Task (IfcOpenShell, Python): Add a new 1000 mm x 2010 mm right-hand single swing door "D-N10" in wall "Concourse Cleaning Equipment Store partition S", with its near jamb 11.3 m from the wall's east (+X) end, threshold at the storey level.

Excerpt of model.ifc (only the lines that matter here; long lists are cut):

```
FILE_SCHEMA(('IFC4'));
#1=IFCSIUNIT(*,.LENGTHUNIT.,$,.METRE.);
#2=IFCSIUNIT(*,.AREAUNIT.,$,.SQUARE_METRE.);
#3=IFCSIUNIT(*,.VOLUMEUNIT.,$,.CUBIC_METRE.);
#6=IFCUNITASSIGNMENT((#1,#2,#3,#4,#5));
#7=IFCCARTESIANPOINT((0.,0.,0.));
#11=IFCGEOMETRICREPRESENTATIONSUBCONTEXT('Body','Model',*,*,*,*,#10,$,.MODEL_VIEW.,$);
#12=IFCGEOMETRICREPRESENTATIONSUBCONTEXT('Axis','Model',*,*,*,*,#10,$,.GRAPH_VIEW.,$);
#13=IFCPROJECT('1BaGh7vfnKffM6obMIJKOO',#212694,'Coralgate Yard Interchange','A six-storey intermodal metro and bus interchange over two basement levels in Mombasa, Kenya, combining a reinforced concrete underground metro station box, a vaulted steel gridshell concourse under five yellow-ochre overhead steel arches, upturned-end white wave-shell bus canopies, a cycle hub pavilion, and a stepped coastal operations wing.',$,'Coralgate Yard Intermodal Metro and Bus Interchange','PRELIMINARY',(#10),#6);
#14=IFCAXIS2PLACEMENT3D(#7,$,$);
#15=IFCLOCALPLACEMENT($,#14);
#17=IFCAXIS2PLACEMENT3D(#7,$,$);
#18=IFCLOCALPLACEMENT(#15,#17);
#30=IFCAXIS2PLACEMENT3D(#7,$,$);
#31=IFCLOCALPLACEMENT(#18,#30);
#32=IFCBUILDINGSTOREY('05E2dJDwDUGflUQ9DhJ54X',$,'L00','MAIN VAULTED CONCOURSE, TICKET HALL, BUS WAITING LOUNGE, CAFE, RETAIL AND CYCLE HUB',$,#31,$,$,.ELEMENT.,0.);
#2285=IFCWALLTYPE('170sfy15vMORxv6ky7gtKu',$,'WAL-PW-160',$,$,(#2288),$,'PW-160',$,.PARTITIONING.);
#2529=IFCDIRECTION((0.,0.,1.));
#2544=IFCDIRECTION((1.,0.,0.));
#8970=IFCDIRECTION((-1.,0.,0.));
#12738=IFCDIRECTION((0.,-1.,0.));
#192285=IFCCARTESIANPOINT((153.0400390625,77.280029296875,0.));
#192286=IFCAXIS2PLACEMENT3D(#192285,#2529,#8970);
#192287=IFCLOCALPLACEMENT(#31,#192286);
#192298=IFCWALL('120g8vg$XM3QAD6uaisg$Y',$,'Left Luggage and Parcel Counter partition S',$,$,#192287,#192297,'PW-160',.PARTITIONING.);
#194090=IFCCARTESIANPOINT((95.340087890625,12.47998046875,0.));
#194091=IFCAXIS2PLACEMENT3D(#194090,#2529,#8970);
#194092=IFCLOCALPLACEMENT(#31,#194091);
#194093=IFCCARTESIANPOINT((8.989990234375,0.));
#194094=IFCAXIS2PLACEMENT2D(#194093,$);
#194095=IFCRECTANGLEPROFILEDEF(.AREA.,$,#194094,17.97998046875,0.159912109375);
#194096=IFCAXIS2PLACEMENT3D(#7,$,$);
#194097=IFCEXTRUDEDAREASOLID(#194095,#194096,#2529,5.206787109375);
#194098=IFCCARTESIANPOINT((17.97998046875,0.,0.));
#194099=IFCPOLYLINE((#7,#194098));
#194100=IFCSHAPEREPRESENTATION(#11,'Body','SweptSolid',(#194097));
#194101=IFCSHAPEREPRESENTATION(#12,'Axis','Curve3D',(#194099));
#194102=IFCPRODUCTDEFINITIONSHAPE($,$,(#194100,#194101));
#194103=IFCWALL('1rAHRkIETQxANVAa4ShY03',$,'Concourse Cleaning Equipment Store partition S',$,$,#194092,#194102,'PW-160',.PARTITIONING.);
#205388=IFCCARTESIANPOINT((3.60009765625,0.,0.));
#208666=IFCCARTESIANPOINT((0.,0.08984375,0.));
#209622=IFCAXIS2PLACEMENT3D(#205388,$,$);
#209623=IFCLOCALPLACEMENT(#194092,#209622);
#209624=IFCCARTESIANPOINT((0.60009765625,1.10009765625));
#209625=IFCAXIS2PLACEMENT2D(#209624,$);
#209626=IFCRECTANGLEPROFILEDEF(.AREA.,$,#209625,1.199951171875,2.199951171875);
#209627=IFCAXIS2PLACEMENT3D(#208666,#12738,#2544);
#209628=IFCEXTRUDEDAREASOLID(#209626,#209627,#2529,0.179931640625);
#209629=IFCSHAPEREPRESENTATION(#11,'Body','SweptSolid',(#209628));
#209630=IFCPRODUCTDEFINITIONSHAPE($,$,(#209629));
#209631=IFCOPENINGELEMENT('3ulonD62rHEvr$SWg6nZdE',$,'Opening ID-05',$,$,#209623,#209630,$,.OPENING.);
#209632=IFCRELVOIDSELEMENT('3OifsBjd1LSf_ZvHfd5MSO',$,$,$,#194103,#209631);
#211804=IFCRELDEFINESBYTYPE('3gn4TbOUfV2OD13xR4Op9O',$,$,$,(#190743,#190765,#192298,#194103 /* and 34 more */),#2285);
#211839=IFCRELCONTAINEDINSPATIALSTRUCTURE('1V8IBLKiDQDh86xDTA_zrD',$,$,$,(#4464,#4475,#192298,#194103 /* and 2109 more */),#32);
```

```python
import numpy as np
import ifcopenshell
import ifcopenshell.api.feature
import ifcopenshell.api.geometry
import ifcopenshell.api.root
import ifcopenshell.api.spatial
import ifcopenshell.geom
import ifcopenshell.util.element
import ifcopenshell.util.placement
import ifcopenshell.util.representation
import ifcopenshell.util.shape
import ifcopenshell.util.unit

model = ifcopenshell.open("model.ifc")
unit_scale = ifcopenshell.util.unit.calculate_unit_scale(model)
settings = ifcopenshell.geom.settings()


def volume(element):
    """Net volume in cubic metres, openings subtracted."""
    shape = ifcopenshell.geom.create_shape(settings, element)
    return ifcopenshell.util.shape.get_volume(shape.geometry)


wall = model.by_id(194103)
storey = ifcopenshell.util.element.get_container(wall, ifc_class="IfcBuildingStorey")
context = ifcopenshell.util.representation.get_context(model, "Model", "Body", "MODEL_VIEW")
before = volume(wall)

width, height, from_end, sill = 1, 2.01, 11.3, 0.0  # metres

# The wall runs along its own X axis, and the end named is its -X end.
wall_shape = ifcopenshell.geom.create_shape(settings, wall)
x, y, z = ifcopenshell.util.shape.get_vertices(wall_shape.geometry).T
start = x.min() + from_end
face, thickness = float(y.min()), float(y.max() - y.min())
wall_matrix = ifcopenshell.util.placement.get_local_placement(wall.ObjectPlacement)
level = ifcopenshell.util.placement.get_local_placement(storey.ObjectPlacement)[2, 3]


def in_wall(x, y):
    """Placement at x, y metres in the wall's axes, at sill height."""
    matrix = wall_matrix.copy()
    matrix[:, 3] = wall_matrix @ np.array([x / unit_scale, y / unit_scale, 0.0, 1.0])
    matrix[2, 3] = level + sill / unit_scale
    return matrix


# Opening: a box that overshoots both wall faces by 50 mm.
opening = ifcopenshell.api.root.create_entity(model, ifc_class="IfcOpeningElement", predefined_type="OPENING")
box = ifcopenshell.api.geometry.add_wall_representation(
    model, context=context, length=width, height=height, thickness=thickness + 0.1
)
ifcopenshell.api.geometry.assign_representation(model, product=opening, representation=box)
ifcopenshell.api.geometry.edit_object_placement(model, product=opening, matrix=in_wall(start, face - 0.05), is_si=False)
ifcopenshell.api.feature.add_feature(model, feature=opening, element=wall)

door = ifcopenshell.api.root.create_entity(model, ifc_class="IfcDoor", name="D-N10", predefined_type="DOOR")
door.OverallWidth, door.OverallHeight = width / unit_scale, height / unit_scale
door.OperationType = "SINGLE_SWING_RIGHT"
body = ifcopenshell.api.geometry.add_door_representation(
    model,
    context=context,
    overall_width=door.OverallWidth,
    overall_height=door.OverallHeight,
    operation_type="SINGLE_SWING_RIGHT",
    lining_properties={"LiningDepth": thickness / unit_scale, "ThresholdDepth": thickness / unit_scale},
)
ifcopenshell.api.geometry.assign_representation(model, product=door, representation=body)
ifcopenshell.api.spatial.assign_container(model, products=[door], relating_structure=storey)
ifcopenshell.api.feature.add_filling(model, opening=opening, element=door)

# The lining spans the wall, so the door starts at the wall face.
ifcopenshell.api.geometry.edit_object_placement(model, product=door, matrix=in_wall(start, face), is_si=False)

after = volume(wall)

print(f"wall volume {before:.3f} -> {after:.3f} m3")

model.write("model_v2.ifc")
```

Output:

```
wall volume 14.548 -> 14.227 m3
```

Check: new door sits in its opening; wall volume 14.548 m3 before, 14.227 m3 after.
